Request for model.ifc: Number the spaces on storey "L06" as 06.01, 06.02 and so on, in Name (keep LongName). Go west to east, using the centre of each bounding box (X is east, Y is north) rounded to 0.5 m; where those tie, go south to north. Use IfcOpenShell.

First a look at what the model holds.

```python
import ifcopenshell
import ifcopenshell.util.element
import ifcopenshell.util.placement

model = ifcopenshell.open("model.ifc")
print(model.schema)
storey = next(s for s in model.by_type("IfcBuildingStorey") if s.Name == "L06")
spaces = [e for e in ifcopenshell.util.element.get_decomposition(storey) if e.is_a("IfcSpace")]
for e in sorted(spaces, key=lambda e: e.id()):
    origin = ifcopenshell.util.placement.get_local_placement(e.ObjectPlacement)[:3, 3]
    print(e.id(), e.Name, e.LongName, origin.round(2) + 0.0, sep=" | ")
```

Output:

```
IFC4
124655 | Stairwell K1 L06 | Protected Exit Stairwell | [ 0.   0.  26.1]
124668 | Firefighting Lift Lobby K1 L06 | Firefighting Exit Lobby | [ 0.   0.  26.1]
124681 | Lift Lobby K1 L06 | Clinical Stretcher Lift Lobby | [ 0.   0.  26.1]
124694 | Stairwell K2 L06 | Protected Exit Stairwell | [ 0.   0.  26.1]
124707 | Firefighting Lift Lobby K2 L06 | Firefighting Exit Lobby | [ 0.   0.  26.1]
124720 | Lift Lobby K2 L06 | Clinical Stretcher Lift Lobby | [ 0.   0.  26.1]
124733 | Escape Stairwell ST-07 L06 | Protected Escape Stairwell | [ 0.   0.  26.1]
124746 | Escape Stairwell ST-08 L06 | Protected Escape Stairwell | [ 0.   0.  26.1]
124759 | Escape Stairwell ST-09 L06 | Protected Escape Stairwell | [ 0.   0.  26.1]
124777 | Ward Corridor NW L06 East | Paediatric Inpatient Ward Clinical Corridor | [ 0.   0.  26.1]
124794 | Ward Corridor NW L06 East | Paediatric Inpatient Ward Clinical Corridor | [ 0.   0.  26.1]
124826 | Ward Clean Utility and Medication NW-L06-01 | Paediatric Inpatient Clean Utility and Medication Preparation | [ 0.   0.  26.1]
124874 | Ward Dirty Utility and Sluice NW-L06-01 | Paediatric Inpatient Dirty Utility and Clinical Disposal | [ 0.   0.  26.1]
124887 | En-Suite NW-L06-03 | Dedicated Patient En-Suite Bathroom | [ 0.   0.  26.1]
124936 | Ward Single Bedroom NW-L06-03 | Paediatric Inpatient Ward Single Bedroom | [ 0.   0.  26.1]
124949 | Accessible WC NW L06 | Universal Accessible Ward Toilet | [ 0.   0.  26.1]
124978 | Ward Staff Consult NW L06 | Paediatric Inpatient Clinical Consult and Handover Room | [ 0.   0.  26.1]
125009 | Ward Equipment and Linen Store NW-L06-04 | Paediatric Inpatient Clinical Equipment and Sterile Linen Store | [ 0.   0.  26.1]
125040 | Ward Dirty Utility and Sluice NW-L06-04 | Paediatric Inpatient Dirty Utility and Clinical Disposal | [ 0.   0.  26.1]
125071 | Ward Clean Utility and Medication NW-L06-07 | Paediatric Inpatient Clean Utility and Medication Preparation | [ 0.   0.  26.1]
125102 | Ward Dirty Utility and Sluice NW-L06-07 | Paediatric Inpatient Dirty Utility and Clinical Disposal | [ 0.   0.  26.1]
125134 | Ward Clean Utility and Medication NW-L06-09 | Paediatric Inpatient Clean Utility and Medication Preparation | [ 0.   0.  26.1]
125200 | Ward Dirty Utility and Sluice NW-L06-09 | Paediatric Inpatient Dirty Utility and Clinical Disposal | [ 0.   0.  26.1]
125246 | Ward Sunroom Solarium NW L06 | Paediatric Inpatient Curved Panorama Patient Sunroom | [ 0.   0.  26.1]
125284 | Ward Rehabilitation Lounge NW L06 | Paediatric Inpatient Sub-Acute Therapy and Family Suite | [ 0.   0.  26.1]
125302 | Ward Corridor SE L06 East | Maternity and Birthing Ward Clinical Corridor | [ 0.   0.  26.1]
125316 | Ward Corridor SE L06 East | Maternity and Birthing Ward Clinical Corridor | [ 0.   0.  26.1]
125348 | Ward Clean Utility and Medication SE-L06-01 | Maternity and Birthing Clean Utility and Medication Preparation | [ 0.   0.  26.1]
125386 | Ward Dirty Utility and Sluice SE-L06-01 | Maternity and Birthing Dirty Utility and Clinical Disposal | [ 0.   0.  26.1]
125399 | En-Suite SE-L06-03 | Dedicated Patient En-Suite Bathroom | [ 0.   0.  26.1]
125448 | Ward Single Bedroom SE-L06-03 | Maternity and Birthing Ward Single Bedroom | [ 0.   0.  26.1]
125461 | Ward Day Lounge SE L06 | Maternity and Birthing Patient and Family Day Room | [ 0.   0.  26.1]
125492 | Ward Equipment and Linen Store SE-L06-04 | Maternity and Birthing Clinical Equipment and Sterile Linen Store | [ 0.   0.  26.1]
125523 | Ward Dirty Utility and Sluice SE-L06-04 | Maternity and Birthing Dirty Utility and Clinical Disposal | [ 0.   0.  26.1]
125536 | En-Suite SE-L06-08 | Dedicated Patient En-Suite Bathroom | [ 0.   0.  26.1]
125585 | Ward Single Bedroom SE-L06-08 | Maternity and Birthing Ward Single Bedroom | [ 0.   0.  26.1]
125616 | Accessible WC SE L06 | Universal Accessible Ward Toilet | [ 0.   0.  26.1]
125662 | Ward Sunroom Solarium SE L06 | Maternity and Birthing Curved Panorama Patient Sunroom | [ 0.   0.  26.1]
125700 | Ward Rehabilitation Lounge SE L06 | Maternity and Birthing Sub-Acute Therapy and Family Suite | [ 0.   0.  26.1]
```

```python
import ifcopenshell
import ifcopenshell.geom
import ifcopenshell.util.element
import ifcopenshell.util.shape

model = ifcopenshell.open("model.ifc")
settings = ifcopenshell.geom.settings()
settings.set("use-world-coords", True)


def centre(element):
    shape = ifcopenshell.geom.create_shape(settings, element)
    return ifcopenshell.util.shape.get_bbox_centroid(shape.geometry)


storey = next(s for s in model.by_type("IfcBuildingStorey") if s.Name == "L06")
spaces = [e for e in ifcopenshell.util.element.get_decomposition(storey) if e.is_a("IfcSpace")]

# Insertion points can sit at a corner or the storey origin, so sort by the geometry (in metres).
centres = {e: centre(e) for e in spaces}
spaces.sort(key=lambda e: (round(centres[e][0] / 0.5), centres[e][1]))

for i, e in enumerate(spaces, start=1):
    number = f"06.{i:02d}"
    e.Name = number
    print(e.id(), number)

model.write("model-out.ifc")
```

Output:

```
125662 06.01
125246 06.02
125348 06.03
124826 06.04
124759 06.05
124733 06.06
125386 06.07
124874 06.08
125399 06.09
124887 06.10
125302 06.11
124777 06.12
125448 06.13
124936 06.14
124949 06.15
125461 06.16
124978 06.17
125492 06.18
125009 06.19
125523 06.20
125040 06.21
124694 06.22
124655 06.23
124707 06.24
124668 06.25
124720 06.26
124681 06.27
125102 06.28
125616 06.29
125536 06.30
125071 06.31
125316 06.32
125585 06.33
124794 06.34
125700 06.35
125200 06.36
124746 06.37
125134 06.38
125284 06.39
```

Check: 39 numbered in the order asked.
